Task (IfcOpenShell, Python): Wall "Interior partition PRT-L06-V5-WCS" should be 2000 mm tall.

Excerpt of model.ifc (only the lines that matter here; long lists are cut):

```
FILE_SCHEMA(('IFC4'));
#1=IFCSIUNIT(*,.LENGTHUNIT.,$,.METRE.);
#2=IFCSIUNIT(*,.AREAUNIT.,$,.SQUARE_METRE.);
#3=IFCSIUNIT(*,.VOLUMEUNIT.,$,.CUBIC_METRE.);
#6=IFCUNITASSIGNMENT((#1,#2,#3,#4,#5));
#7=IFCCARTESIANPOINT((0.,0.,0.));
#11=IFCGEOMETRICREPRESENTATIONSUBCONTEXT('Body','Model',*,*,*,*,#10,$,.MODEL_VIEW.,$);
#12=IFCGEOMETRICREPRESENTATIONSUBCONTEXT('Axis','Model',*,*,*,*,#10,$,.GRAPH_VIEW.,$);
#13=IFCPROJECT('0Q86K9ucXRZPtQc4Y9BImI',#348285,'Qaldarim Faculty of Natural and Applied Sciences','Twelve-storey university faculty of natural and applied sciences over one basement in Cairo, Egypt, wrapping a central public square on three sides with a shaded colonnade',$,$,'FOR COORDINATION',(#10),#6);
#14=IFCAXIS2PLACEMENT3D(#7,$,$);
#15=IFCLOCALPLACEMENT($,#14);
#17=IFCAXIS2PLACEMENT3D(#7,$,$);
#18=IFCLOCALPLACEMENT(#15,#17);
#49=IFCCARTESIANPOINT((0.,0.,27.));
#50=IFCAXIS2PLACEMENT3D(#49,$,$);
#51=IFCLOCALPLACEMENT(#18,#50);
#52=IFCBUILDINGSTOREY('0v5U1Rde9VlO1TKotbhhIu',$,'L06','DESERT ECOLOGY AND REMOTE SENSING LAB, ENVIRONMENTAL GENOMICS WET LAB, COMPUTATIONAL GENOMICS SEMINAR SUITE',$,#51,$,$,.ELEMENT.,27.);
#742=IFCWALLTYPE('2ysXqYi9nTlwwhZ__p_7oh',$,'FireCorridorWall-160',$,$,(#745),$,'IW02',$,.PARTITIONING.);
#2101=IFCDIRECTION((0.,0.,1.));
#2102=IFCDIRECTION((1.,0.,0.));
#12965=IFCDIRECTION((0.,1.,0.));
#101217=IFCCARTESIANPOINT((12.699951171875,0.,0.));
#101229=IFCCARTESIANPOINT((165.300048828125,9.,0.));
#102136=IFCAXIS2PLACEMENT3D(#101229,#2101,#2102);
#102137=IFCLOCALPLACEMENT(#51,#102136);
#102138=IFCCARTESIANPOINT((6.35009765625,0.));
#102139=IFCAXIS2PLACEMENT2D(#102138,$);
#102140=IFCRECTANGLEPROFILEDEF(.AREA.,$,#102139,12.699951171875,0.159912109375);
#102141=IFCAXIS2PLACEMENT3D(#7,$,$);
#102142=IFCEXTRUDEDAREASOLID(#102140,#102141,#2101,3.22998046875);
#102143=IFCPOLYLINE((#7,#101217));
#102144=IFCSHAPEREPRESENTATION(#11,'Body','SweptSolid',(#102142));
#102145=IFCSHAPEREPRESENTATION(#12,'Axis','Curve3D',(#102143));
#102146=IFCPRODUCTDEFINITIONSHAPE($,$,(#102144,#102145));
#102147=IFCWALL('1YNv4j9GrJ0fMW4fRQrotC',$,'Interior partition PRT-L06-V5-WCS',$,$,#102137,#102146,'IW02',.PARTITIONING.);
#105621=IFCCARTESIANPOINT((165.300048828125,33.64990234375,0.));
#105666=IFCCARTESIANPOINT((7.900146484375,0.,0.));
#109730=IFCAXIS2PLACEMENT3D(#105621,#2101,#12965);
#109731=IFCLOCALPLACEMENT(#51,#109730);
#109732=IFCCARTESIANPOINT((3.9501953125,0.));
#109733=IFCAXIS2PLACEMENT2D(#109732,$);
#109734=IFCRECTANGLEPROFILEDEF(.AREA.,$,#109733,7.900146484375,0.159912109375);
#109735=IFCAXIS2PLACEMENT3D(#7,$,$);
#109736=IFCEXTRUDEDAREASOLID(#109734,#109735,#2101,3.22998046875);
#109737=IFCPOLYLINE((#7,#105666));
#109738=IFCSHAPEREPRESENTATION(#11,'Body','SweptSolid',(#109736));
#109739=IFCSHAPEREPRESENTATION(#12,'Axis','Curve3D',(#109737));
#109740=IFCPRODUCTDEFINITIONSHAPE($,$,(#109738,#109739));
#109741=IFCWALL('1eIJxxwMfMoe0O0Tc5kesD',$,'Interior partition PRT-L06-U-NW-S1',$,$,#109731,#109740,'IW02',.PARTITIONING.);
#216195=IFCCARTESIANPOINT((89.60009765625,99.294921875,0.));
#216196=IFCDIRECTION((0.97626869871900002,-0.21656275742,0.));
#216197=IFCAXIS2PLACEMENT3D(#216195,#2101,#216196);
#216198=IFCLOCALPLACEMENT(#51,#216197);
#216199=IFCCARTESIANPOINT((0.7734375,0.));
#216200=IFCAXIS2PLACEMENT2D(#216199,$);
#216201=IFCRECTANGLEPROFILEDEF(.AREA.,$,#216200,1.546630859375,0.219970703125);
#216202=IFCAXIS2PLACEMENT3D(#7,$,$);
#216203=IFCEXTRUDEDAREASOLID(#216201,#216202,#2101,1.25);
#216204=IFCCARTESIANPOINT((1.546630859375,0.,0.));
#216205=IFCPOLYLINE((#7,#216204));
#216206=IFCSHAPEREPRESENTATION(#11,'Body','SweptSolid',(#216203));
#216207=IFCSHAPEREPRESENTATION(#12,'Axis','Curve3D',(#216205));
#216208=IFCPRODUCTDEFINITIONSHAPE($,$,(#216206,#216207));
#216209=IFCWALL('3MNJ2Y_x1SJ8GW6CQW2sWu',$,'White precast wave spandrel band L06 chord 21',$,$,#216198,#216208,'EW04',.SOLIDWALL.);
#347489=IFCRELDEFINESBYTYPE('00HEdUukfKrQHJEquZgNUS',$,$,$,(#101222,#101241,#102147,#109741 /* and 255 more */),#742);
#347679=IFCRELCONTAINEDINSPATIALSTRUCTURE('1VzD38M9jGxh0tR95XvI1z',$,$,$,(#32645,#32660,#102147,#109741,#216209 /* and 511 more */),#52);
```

```python
import ifcopenshell
import ifcopenshell.geom
import ifcopenshell.util.representation
import ifcopenshell.util.shape
import ifcopenshell.util.unit

model = ifcopenshell.open("model.ifc")
unit_scale = ifcopenshell.util.unit.calculate_unit_scale(model)
settings = ifcopenshell.geom.settings()


def volume(element):
    """Net volume in cubic metres, openings subtracted."""
    shape = ifcopenshell.geom.create_shape(settings, element)
    return ifcopenshell.util.shape.get_volume(shape.geometry)


wall = model.by_guid("1YNv4j9GrJ0fMW4fRQrotC")
before = volume(wall)

body = ifcopenshell.util.representation.get_representation(wall, "Model", "Body")
solid = body.Items[0]
old_height = solid.Depth
solid.Depth = 2 / unit_scale
after = volume(wall)

print(f"height {old_height:g} -> {solid.Depth:g}, volume {before:.3f} -> {after:.3f} m3")

model.write("model_edited.ifc")
```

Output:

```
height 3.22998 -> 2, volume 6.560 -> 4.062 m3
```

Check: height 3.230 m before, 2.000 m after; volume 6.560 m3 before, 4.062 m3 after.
